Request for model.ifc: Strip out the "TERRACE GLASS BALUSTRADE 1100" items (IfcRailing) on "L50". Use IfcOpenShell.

First a look at what the model holds.

```python
import ifcopenshell
import ifcopenshell.util.element

model = ifcopenshell.open("model.ifc")
print(model.schema)
storey = next(s for s in model.by_type("IfcBuildingStorey") if s.Name == "L50")
railings = [e for e in ifcopenshell.util.element.get_decomposition(storey) if e.is_a("IfcRailing")]
seen = {}
for e in railings:
    element_type = ifcopenshell.util.element.get_type(e)
    name = element_type.Name if element_type not in (None, e) else None
    seen[name] = seen.get(name, 0) + 1
for name, count in sorted(seen.items(), key=str):
    print(count, "x", name)
```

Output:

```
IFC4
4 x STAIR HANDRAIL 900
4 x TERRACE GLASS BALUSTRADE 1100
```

```python
import ifcopenshell
import ifcopenshell.api.root
import ifcopenshell.util.element

model = ifcopenshell.open("model.ifc")

storey = next(s for s in model.by_type("IfcBuildingStorey") if s.Name == "L50")
railings = [e for e in ifcopenshell.util.element.get_decomposition(storey) if e.is_a("IfcRailing")]
targets = [e for e in railings if (t := ifcopenshell.util.element.get_type(e)) not in (None, e) and t.Name == "TERRACE GLASS BALUSTRADE 1100"]

for e in targets:
    ifcopenshell.api.root.remove_product(model, product=e)
print(len(targets), "removed")

model.write("model-out.ifc")
```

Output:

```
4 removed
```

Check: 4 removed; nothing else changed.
